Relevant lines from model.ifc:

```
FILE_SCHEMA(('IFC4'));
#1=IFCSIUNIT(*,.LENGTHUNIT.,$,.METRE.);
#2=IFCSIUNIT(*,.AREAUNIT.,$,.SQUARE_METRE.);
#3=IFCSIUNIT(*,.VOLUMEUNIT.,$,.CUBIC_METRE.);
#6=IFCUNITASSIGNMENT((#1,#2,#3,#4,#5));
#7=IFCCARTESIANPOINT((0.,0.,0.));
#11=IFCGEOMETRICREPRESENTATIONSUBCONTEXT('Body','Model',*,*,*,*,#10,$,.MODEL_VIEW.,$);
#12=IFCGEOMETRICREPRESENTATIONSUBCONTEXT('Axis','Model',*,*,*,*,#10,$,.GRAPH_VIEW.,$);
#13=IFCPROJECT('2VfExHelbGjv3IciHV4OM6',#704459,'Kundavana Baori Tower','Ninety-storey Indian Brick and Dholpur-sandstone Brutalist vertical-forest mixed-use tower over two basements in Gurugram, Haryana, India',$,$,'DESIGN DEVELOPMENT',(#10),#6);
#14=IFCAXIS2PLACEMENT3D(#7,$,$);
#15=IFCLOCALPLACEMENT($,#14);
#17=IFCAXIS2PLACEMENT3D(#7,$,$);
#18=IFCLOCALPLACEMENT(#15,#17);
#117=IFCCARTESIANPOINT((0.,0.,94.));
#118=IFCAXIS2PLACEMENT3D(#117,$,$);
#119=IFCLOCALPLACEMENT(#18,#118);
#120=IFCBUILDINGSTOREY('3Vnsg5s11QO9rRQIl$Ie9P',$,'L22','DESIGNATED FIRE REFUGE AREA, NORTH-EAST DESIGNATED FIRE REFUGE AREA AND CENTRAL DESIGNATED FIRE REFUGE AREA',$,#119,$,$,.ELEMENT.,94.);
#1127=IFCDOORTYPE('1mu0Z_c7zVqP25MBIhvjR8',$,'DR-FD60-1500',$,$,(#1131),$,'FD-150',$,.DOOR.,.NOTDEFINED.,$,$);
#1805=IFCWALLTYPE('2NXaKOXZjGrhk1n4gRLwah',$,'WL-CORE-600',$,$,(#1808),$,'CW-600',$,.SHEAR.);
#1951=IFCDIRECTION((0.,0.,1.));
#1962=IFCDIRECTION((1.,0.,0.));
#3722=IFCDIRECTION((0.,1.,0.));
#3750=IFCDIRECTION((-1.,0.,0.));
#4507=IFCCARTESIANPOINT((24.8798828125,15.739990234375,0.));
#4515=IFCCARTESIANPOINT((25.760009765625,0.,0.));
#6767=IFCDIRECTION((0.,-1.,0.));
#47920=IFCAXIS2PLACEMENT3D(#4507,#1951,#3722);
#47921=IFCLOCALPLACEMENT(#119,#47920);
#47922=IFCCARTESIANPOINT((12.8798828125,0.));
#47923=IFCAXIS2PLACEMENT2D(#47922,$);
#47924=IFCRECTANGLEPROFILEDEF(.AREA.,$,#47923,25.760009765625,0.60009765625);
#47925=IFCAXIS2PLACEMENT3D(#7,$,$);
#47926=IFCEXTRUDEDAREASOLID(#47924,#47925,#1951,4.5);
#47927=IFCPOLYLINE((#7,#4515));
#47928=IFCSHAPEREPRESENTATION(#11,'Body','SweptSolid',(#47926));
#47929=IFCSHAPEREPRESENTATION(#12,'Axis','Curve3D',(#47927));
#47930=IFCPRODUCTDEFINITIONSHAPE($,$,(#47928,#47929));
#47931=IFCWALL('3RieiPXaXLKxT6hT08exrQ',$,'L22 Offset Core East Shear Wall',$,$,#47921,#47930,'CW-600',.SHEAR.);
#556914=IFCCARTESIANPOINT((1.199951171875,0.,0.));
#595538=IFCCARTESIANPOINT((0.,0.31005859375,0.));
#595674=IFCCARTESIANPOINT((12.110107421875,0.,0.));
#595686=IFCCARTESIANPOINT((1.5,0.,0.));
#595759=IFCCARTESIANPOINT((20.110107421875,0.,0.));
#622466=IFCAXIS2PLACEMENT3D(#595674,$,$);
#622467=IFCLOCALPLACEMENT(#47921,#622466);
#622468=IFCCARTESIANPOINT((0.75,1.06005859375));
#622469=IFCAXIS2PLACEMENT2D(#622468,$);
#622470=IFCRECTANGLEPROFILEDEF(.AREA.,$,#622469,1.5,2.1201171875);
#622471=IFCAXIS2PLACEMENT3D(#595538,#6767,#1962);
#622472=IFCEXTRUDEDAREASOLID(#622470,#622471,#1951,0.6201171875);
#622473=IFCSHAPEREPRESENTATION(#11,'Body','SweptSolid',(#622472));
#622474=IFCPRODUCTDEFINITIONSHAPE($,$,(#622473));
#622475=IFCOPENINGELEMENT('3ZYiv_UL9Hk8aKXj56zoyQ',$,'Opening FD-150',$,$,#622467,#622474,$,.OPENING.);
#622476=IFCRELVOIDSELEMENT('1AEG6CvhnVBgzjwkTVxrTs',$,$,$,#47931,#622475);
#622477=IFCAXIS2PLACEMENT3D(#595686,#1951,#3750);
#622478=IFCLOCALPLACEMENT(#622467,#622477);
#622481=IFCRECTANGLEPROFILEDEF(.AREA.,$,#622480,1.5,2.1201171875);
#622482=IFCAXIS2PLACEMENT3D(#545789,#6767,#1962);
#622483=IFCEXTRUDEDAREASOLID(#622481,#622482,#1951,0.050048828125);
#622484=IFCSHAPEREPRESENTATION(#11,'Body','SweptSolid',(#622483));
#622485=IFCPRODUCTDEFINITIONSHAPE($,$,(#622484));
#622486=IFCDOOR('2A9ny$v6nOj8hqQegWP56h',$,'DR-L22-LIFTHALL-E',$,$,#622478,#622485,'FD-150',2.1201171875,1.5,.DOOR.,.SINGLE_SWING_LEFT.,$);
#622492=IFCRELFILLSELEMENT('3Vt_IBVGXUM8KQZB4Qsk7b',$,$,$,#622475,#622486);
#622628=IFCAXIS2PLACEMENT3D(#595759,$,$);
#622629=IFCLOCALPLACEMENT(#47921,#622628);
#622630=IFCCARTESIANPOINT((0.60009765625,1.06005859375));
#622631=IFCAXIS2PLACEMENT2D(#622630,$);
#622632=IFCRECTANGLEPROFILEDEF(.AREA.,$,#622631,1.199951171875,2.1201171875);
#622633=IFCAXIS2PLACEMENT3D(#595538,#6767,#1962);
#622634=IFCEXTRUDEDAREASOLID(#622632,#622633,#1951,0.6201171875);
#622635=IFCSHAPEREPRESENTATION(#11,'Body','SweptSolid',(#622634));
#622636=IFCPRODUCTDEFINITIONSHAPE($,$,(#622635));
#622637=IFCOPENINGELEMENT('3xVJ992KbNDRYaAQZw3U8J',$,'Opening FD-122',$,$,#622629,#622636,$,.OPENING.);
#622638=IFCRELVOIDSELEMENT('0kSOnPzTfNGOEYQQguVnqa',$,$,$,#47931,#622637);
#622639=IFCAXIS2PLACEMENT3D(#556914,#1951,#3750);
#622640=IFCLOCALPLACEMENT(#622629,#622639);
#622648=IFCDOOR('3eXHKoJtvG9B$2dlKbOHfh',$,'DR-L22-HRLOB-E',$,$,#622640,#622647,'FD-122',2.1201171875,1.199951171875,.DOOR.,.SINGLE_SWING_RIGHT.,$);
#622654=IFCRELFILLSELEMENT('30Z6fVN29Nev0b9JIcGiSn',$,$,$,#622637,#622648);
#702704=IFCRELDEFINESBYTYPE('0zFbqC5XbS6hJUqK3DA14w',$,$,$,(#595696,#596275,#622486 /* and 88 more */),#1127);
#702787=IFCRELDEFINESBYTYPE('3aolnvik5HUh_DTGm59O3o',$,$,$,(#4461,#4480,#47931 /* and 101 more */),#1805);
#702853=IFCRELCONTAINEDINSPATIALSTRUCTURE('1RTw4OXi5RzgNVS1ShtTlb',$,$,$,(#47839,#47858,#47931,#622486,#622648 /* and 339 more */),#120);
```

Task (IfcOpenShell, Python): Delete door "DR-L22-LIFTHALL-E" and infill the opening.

```python
import ifcopenshell
import ifcopenshell.api.feature
import ifcopenshell.api.root
import ifcopenshell.geom
import ifcopenshell.util.shape

model = ifcopenshell.open("model.ifc")
settings = ifcopenshell.geom.settings()


def volume(element):
    """Net volume in cubic metres, openings subtracted."""
    shape = ifcopenshell.geom.create_shape(settings, element)
    return ifcopenshell.util.shape.get_volume(shape.geometry)


door = model.by_guid("2A9ny$v6nOj8hqQegWP56h")
opening = door.FillsVoids[0].RelatingOpeningElement
wall = opening.VoidsElements[0].RelatingBuildingElement
before = volume(wall)

ifcopenshell.api.root.remove_product(model, product=door)
ifcopenshell.api.feature.remove_feature(model, feature=opening)

after = volume(wall)

print(f"wall volume {before:.3f} -> {after:.3f} m3")

model.write("model_updated.ifc")
```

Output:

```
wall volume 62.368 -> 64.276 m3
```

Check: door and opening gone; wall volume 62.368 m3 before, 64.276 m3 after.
